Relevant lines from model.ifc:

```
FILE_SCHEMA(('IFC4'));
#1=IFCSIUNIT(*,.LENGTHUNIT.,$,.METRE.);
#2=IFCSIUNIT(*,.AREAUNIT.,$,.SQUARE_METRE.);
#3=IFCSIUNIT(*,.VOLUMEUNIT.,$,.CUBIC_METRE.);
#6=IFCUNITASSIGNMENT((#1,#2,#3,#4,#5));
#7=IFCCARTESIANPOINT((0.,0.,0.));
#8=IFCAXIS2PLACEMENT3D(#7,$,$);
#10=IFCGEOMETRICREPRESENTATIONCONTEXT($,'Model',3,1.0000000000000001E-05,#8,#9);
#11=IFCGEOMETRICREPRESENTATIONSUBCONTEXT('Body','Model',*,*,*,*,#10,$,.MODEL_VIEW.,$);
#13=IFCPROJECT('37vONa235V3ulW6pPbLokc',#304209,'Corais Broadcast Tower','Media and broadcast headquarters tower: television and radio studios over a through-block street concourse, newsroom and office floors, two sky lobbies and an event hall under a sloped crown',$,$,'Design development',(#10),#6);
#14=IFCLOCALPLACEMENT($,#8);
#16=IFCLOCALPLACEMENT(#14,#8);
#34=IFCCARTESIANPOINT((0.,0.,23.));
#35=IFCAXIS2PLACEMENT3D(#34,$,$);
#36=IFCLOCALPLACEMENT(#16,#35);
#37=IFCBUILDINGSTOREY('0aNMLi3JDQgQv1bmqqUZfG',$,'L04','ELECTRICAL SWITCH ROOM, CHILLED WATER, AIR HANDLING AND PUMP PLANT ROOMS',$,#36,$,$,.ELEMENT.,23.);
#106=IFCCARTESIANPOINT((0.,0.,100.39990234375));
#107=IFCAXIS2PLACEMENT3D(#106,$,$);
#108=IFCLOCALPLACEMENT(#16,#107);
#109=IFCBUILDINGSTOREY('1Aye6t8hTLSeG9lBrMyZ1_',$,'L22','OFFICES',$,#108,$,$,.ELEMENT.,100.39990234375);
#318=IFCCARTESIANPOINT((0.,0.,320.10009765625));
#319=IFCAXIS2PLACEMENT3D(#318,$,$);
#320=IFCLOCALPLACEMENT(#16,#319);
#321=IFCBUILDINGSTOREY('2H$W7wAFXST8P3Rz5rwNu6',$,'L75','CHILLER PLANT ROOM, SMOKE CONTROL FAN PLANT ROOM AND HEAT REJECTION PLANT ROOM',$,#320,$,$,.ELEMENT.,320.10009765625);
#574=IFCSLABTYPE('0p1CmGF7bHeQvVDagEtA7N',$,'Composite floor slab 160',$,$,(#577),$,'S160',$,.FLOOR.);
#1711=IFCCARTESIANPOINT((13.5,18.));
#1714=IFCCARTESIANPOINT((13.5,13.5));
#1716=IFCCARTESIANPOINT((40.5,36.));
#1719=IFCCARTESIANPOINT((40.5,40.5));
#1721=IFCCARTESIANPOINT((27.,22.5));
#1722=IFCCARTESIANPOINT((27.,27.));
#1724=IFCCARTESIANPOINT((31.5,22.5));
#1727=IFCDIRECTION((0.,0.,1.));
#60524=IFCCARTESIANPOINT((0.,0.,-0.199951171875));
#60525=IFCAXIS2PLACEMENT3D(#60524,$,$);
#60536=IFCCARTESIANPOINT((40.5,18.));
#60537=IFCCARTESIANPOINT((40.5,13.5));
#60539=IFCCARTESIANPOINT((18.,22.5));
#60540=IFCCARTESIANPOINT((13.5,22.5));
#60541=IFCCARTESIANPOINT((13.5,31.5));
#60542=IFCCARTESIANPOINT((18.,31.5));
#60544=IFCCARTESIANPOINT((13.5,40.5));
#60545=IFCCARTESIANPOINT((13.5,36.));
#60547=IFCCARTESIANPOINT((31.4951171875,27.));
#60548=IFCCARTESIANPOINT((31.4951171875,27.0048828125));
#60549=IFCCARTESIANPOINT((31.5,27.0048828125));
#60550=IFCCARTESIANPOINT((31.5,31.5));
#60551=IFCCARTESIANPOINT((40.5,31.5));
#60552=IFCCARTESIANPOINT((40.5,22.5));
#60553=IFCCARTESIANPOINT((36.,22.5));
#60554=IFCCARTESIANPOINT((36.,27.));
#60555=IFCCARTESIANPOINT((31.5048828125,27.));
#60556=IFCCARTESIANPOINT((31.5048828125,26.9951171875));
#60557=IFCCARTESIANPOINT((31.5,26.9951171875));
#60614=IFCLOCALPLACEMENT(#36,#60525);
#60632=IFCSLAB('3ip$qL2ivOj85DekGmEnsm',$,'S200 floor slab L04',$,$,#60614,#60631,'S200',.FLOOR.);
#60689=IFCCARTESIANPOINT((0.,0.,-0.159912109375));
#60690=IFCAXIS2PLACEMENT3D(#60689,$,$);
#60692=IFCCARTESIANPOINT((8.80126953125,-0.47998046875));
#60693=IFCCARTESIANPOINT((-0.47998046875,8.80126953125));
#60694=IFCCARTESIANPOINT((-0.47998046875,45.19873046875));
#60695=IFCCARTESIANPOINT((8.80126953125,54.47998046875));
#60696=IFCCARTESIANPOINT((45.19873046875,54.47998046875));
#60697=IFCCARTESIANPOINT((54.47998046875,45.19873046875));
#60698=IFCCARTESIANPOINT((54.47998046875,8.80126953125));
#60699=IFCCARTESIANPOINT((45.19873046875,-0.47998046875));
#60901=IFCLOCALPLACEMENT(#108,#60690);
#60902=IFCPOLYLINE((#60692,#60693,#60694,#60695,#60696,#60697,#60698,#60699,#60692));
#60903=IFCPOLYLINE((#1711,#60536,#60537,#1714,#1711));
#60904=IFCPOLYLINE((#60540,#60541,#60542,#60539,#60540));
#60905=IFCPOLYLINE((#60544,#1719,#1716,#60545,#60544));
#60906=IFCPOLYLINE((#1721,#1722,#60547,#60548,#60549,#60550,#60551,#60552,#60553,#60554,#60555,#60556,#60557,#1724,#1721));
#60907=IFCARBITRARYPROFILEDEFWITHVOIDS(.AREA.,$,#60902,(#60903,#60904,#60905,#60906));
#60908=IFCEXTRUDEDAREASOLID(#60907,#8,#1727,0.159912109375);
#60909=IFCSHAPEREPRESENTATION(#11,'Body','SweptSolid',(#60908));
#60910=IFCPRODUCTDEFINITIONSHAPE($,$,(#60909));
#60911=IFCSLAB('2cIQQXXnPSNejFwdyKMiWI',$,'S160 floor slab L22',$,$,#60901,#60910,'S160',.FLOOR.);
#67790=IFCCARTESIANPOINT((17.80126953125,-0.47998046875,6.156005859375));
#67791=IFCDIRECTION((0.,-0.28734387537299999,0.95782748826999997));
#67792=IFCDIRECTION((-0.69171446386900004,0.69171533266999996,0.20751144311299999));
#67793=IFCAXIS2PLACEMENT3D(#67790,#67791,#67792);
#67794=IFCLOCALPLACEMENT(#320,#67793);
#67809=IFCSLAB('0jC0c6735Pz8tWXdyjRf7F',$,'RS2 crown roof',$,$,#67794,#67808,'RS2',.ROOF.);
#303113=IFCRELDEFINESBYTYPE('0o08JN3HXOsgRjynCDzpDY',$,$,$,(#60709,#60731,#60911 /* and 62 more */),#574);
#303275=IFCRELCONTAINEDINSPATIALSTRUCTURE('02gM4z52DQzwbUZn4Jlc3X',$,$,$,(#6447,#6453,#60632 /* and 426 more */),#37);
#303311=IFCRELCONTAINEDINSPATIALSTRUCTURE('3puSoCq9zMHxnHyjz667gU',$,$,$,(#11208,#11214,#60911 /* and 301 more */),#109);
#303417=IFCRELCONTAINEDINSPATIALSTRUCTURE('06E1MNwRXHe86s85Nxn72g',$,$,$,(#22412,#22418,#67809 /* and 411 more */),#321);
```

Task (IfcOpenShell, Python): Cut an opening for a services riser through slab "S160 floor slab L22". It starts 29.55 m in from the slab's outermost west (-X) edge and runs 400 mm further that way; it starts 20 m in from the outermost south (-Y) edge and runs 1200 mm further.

```python
import numpy as np
import ifcopenshell
import ifcopenshell.api.feature
import ifcopenshell.api.geometry
import ifcopenshell.api.root
import ifcopenshell.geom
import ifcopenshell.util.placement
import ifcopenshell.util.representation
import ifcopenshell.util.shape
import ifcopenshell.util.unit

model = ifcopenshell.open("model.ifc")
unit_scale = ifcopenshell.util.unit.calculate_unit_scale(model)
settings = ifcopenshell.geom.settings()


def volume(element):
    """Net volume in cubic metres, openings subtracted."""
    shape = ifcopenshell.geom.create_shape(settings, element)
    return ifcopenshell.util.shape.get_volume(shape.geometry)


slab = model.by_guid("2cIQQXXnPSNejFwdyKMiWI")
before = volume(slab)

# Extent in the slab's own axes, in metres. The edges named are its -X and -Y sides.
slab_shape = ifcopenshell.geom.create_shape(settings, slab)
vertices = ifcopenshell.util.shape.get_vertices(slab_shape.geometry)
x_min, y_min, bottom = vertices.min(axis=0)
top = vertices[:, 2].max()

opening = ifcopenshell.api.root.create_entity(model, ifc_class="IfcOpeningElement", name="Services riser opening", predefined_type="OPENING")
context = ifcopenshell.util.representation.get_context(model, "Model", "Body", "MODEL_VIEW")
width, depth = 0.4, 1.2
outline = [(0.0, 0.0), (width, 0.0), (width, depth), (0.0, depth), (0.0, 0.0)]
# Overshoot both faces by 50 mm so the cut is clean.
shape = ifcopenshell.api.geometry.add_slab_representation(
    model, context=context, depth=top - bottom + 0.1, polyline=outline
)
ifcopenshell.api.geometry.assign_representation(model, product=opening, representation=shape)

matrix = ifcopenshell.util.placement.get_local_placement(slab.ObjectPlacement)
matrix[:, 3] = matrix @ np.append(np.array([x_min + 29.55, y_min + 20, bottom - 0.05]) / unit_scale, 1.0)
ifcopenshell.api.geometry.edit_object_placement(model, product=opening, matrix=matrix, is_si=False)
ifcopenshell.api.feature.add_feature(model, feature=opening, element=slab)

after = volume(slab)

print(f"slab volume {before:.3f} -> {after:.3f} m3")

model.write("model-out.ifc")
```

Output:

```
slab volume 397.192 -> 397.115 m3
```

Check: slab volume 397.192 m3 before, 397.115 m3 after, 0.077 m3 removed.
